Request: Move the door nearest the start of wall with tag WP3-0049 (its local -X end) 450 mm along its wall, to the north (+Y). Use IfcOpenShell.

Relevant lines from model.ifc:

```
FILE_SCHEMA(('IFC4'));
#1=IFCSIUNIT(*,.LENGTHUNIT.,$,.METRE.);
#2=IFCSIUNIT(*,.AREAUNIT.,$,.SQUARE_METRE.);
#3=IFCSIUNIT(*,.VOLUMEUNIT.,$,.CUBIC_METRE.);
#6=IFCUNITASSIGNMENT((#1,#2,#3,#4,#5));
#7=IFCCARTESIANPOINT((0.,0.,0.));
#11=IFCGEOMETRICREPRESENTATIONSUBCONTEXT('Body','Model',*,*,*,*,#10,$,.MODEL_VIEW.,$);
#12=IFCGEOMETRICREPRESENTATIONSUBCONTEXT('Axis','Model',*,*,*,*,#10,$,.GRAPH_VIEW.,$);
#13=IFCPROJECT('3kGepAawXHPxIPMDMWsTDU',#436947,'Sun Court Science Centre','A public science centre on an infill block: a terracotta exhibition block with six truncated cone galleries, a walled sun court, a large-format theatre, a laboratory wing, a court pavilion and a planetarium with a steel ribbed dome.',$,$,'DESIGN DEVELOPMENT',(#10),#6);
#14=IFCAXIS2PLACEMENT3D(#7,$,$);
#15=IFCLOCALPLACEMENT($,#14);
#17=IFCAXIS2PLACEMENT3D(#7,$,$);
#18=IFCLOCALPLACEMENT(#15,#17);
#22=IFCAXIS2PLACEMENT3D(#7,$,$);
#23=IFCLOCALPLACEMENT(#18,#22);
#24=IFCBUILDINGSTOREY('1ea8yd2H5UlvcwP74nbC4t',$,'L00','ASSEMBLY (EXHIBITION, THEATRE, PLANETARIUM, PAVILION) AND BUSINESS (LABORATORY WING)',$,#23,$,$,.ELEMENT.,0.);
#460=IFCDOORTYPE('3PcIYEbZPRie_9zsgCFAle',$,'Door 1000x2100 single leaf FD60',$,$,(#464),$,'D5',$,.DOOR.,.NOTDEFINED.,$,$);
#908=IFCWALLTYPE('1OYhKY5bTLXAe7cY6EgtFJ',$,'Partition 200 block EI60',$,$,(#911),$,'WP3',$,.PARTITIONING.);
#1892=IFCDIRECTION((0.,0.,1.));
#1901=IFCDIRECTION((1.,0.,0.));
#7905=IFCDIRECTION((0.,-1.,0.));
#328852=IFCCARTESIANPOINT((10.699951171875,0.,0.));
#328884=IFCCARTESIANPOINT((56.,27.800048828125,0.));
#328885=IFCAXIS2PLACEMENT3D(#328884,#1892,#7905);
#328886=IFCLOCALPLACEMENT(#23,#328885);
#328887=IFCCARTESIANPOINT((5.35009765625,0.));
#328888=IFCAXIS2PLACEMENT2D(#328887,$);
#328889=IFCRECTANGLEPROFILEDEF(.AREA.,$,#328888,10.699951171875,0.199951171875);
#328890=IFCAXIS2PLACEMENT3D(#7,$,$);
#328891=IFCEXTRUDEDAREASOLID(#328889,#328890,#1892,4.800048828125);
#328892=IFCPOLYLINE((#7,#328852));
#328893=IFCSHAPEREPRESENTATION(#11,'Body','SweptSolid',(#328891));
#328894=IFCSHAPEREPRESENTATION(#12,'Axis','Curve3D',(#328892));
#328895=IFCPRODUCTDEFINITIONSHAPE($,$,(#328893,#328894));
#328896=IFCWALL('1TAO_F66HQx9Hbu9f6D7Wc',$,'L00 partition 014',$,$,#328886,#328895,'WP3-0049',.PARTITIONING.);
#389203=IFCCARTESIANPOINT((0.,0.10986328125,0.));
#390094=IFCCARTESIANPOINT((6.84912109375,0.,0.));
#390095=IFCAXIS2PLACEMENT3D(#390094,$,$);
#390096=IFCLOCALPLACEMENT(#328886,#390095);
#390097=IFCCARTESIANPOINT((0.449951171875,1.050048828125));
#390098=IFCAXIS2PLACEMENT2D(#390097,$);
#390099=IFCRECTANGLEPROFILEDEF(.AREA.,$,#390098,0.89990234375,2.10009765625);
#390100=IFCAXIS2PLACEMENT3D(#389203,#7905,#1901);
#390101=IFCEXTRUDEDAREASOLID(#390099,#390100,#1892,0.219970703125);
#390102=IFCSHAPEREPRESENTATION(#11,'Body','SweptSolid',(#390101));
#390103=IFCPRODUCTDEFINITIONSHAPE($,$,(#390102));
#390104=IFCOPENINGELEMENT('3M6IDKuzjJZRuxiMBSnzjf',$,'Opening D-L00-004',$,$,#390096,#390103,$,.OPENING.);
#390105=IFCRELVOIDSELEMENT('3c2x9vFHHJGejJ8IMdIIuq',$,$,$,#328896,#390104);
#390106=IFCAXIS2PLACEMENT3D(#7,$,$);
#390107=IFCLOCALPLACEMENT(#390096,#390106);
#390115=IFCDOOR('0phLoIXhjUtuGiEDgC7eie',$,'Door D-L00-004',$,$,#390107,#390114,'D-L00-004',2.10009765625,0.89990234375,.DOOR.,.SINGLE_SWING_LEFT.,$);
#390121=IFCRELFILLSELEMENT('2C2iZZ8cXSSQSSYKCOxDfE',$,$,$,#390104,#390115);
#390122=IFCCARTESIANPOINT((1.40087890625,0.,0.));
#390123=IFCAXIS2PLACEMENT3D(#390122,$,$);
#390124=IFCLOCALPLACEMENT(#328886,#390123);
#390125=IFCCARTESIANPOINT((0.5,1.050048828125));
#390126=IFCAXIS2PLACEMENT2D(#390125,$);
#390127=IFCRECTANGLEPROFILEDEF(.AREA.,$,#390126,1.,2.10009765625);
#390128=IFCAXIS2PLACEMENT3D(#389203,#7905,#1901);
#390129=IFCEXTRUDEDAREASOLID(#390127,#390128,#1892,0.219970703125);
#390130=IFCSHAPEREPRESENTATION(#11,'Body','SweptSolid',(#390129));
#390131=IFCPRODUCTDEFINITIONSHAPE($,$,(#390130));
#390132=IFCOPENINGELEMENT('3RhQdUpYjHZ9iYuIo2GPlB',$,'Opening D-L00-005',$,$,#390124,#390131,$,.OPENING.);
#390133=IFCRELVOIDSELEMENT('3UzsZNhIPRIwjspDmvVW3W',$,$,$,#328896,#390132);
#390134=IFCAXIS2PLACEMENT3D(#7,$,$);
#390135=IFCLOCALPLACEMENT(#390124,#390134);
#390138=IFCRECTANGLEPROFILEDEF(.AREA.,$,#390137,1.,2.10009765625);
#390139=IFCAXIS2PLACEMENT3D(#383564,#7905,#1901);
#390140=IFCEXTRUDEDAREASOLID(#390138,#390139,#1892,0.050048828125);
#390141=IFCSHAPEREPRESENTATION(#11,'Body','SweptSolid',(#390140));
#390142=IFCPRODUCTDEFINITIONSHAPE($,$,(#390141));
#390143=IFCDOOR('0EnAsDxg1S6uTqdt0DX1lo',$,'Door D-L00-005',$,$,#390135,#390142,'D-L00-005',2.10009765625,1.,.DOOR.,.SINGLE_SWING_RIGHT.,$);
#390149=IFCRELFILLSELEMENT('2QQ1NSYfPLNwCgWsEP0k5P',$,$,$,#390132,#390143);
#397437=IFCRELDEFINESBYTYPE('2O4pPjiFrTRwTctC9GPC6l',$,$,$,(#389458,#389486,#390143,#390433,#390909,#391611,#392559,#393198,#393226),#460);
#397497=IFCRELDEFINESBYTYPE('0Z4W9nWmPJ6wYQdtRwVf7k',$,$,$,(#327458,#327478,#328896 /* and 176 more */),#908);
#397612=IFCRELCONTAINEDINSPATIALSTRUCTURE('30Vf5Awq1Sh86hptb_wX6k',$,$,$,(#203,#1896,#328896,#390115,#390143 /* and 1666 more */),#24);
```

```python
import ifcopenshell
import ifcopenshell.api.geometry
import ifcopenshell.util.placement
import ifcopenshell.util.unit

model = ifcopenshell.open("model.ifc")
unit_scale = ifcopenshell.util.unit.calculate_unit_scale(model)

door = model.by_guid("0EnAsDxg1S6uTqdt0DX1lo")
opening = door.FillsVoids[0].RelatingOpeningElement
wall = opening.VoidsElements[0].RelatingBuildingElement

wall_matrix = ifcopenshell.util.placement.get_local_placement(wall.ObjectPlacement)
shift = wall_matrix[:3, 0] * -0.45 / unit_scale
before = ifcopenshell.util.placement.get_local_placement(door.ObjectPlacement)[:3, 3].copy()

# The door is placed relative to its opening, so it follows when the opening moves.
matrix = ifcopenshell.util.placement.get_local_placement(opening.ObjectPlacement)
matrix[:3, 3] += shift
ifcopenshell.api.geometry.edit_object_placement(
    model, product=opening, matrix=matrix, is_si=False, should_transform_children=True
)

after = ifcopenshell.util.placement.get_local_placement(door.ObjectPlacement)[:3, 3]
print("door moved by", (after - before).round(3) + 0.0)

model.write("model_v2.ifc")
```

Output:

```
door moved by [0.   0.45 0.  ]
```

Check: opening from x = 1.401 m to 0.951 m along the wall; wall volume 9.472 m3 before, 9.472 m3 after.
